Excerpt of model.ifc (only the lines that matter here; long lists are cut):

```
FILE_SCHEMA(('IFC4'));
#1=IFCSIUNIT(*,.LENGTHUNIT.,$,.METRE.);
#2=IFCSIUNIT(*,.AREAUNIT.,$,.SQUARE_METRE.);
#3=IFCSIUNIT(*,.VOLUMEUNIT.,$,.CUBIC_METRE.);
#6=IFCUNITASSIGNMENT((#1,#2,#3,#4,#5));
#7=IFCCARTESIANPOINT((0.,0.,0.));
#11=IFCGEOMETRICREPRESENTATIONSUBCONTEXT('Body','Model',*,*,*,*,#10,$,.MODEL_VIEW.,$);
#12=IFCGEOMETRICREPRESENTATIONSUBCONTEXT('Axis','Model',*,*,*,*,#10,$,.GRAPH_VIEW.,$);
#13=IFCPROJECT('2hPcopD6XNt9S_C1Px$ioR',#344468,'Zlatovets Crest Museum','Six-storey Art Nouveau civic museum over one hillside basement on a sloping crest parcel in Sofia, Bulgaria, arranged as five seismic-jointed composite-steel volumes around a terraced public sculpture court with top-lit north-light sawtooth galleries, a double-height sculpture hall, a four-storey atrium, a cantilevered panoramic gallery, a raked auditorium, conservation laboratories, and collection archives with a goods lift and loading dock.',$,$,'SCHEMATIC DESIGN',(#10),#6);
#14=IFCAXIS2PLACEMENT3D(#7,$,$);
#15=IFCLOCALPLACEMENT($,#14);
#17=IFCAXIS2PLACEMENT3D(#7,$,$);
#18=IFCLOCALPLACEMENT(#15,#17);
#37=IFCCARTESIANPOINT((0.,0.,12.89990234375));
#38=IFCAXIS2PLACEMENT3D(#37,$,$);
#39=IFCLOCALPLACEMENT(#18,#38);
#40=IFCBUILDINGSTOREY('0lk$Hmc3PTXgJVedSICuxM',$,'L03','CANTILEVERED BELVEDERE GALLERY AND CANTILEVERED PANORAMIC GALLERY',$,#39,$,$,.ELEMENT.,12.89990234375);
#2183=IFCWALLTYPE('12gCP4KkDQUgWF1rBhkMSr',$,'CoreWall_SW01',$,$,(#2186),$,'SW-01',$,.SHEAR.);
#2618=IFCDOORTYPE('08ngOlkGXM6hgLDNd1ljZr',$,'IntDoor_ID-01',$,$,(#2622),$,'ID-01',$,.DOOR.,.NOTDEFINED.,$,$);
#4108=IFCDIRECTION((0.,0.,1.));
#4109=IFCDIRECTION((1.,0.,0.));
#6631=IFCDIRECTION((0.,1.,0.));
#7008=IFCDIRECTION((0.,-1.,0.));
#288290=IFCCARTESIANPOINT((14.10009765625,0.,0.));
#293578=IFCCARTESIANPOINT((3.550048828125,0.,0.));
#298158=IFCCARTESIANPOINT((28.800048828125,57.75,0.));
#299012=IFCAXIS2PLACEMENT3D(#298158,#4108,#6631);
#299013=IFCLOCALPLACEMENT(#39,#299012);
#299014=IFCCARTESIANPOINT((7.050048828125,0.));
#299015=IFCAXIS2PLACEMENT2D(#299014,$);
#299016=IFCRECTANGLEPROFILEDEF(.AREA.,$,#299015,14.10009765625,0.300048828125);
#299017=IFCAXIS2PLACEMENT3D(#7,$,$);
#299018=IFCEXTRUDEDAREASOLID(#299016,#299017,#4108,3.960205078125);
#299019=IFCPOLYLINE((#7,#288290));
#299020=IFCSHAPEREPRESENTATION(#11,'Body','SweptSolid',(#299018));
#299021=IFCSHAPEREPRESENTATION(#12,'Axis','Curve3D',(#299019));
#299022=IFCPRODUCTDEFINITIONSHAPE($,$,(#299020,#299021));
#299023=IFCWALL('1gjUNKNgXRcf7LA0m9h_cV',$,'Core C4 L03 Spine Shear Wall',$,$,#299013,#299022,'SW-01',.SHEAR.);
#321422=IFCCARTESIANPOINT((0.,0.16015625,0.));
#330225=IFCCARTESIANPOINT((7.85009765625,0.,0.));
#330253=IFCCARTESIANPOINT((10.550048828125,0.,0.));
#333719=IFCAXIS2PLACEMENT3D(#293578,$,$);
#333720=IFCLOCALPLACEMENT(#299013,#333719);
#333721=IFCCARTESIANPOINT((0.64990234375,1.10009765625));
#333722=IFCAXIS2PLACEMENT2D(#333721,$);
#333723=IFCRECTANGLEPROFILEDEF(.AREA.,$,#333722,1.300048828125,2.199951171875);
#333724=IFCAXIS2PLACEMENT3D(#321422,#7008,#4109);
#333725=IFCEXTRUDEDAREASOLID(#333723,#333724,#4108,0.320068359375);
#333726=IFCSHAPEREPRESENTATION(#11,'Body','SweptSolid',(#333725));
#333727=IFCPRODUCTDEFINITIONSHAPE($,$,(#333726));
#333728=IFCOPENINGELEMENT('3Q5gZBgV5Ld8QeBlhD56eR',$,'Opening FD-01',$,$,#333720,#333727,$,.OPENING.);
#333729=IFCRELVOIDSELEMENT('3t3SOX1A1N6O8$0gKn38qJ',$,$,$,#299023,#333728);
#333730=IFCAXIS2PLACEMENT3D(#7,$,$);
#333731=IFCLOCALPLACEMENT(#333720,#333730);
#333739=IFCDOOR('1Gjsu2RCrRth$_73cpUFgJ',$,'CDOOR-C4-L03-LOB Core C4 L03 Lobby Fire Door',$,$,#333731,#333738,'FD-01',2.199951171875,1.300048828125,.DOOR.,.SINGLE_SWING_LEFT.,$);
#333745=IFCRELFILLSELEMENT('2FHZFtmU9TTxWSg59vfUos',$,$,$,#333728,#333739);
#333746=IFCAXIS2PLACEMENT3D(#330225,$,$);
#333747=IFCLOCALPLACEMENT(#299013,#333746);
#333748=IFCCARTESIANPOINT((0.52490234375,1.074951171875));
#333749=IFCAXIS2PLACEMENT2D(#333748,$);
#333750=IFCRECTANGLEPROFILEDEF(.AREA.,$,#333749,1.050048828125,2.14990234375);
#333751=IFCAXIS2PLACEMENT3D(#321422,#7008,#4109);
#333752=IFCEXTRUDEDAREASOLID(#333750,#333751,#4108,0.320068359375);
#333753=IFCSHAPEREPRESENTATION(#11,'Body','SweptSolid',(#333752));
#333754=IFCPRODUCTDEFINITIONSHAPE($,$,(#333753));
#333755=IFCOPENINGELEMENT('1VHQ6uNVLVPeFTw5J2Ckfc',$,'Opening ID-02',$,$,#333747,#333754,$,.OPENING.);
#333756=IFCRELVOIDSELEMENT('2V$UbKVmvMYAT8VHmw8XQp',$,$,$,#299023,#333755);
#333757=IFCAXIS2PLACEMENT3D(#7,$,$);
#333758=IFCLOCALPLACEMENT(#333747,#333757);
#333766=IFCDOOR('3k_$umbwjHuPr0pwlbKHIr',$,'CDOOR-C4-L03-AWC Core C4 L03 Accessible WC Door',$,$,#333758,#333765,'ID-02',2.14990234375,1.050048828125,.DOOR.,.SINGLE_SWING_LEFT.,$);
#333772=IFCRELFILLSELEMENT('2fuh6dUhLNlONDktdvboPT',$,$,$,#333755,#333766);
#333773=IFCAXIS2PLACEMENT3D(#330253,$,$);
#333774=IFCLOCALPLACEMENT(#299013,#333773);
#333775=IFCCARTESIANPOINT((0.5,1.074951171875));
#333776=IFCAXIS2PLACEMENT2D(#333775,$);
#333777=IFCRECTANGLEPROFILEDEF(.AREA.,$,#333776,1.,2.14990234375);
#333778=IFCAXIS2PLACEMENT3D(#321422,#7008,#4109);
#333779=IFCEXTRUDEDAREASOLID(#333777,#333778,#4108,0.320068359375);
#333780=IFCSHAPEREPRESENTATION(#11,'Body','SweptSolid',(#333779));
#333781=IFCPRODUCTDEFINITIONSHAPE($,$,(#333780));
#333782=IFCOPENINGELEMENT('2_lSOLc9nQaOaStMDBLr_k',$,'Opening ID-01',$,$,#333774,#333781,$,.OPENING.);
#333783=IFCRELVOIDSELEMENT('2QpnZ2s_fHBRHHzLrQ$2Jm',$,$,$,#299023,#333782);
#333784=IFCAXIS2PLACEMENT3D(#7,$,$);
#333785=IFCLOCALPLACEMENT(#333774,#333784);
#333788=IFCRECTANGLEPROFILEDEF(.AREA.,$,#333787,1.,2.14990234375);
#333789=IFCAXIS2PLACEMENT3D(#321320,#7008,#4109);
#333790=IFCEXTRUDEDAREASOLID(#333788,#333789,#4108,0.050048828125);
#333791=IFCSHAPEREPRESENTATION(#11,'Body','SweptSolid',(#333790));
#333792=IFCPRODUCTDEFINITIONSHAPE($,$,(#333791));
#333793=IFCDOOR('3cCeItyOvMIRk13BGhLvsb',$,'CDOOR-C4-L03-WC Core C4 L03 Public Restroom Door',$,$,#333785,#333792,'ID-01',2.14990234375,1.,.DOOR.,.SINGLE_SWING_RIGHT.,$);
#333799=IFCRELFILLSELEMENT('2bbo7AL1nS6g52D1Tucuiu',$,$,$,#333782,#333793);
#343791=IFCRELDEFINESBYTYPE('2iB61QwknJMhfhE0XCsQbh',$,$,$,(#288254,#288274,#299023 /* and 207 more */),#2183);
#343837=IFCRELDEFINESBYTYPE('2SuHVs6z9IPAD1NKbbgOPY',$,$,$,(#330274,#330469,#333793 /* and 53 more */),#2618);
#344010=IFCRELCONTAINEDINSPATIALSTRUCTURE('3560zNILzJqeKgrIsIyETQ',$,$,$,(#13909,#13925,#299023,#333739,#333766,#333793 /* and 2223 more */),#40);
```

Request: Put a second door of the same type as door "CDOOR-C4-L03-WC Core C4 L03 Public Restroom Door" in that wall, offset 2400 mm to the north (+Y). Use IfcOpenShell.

```python
import ifcopenshell
import ifcopenshell.api.feature
import ifcopenshell.api.geometry
import ifcopenshell.api.root
import ifcopenshell.geom
import ifcopenshell.util.element
import ifcopenshell.util.placement
import ifcopenshell.util.shape

model = ifcopenshell.open("model.ifc")
settings = ifcopenshell.geom.settings()


def volume(element):
    """Net volume in cubic metres, openings subtracted."""
    shape = ifcopenshell.geom.create_shape(settings, element)
    return ifcopenshell.util.shape.get_volume(shape.geometry)


door = model.by_guid("3cCeItyOvMIRk13BGhLvsb")
opening = door.FillsVoids[0].RelatingOpeningElement
wall = opening.VoidsElements[0].RelatingBuildingElement
before = volume(wall)
shift = ifcopenshell.util.placement.get_local_placement(wall.ObjectPlacement)[:3, 0] * 2.4

# copy_class copies the void relationship, type, container and properties, but no geometry.
new_opening = ifcopenshell.api.root.copy_class(model, product=opening)
new_opening.Representation = ifcopenshell.util.element.copy_deep(
    model, opening.Representation, exclude=["IfcGeometricRepresentationContext", "IfcRepresentationMap"]
)
new_door = ifcopenshell.api.root.copy_class(model, product=door)
new_door.Representation = ifcopenshell.util.element.copy_deep(
    model, door.Representation, exclude=["IfcGeometricRepresentationContext", "IfcRepresentationMap"]
)
new_door.Tag = None
ifcopenshell.api.feature.add_filling(model, opening=new_opening, element=new_door)

for old, new in ((opening, new_opening), (door, new_door)):
    matrix = ifcopenshell.util.placement.get_local_placement(old.ObjectPlacement)
    matrix[:3, 3] += shift
    ifcopenshell.api.geometry.edit_object_placement(model, product=new, matrix=matrix, is_si=False)

after = volume(wall)

print(f"wall volume {before:.3f} -> {after:.3f} m3")

model.write("model_rev.ifc")
```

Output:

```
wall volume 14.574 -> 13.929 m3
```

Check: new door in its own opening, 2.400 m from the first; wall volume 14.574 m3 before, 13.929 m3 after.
